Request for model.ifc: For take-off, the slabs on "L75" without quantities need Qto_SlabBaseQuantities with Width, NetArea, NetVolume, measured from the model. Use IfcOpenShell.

First a look at what the model holds.

```python
import ifcopenshell
import ifcopenshell.util.element
import ifcopenshell.util.unit

model = ifcopenshell.open("model.ifc")
print(model.schema)
for unit_type in ("LENGTHUNIT", "AREAUNIT", "VOLUMEUNIT"):
    print(unit_type, ifcopenshell.util.unit.calculate_unit_scale(model, unit_type))
storey = next(s for s in model.by_type("IfcBuildingStorey") if s.Name == "L75")
slabs = [e for e in ifcopenshell.util.element.get_decomposition(storey) if e.is_a("IfcSlab")]
for e in sorted(slabs, key=lambda e: e.id()):
    print(e.id(), e.is_a(), e.Name, list(ifcopenshell.util.element.get_psets(e, qtos_only=True)), sep=" | ")
```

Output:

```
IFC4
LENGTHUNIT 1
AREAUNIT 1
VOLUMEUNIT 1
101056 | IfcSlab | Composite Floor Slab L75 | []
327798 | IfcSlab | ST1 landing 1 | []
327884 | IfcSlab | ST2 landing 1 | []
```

```python
import ifcopenshell
import ifcopenshell.api.pset
import ifcopenshell.geom
import ifcopenshell.util.element
import ifcopenshell.util.shape
import ifcopenshell.util.unit

model = ifcopenshell.open("model.ifc")
unit_scale = ifcopenshell.util.unit.calculate_unit_scale(model)
area_scale = ifcopenshell.util.unit.calculate_unit_scale(model, "AREAUNIT")
volume_scale = ifcopenshell.util.unit.calculate_unit_scale(model, "VOLUMEUNIT")
settings = ifcopenshell.geom.settings()

storey = next(s for s in model.by_type("IfcBuildingStorey") if s.Name == "L75")
slabs = [e for e in ifcopenshell.util.element.get_decomposition(storey) if e.is_a("IfcSlab")]

for e in sorted(slabs, key=lambda e: e.id()):
    if ifcopenshell.util.element.get_psets(e, qtos_only=True, should_inherit=False):
        continue
    # Geometry comes back in metres, in the element's own axes.
    shape = ifcopenshell.geom.create_shape(settings, e)
    values = {
        "Width": ifcopenshell.util.shape.get_z(shape.geometry) / unit_scale,
        "NetArea": ifcopenshell.util.shape.get_footprint_area(shape.geometry) / area_scale,
        "NetVolume": ifcopenshell.util.shape.get_volume(shape.geometry) / volume_scale,
    }
    qto = ifcopenshell.api.pset.add_qto(model, product=e, name="Qto_SlabBaseQuantities")
    ifcopenshell.api.pset.edit_qto(model, qto=qto, properties=values)
    print(e.id(), {k: round(v, 3) for k, v in values.items()})

model.write("model_edited.ifc")
```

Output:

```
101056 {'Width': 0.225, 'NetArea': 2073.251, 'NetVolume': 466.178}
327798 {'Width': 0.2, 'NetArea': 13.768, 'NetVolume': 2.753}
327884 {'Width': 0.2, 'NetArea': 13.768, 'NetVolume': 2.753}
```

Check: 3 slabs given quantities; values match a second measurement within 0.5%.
